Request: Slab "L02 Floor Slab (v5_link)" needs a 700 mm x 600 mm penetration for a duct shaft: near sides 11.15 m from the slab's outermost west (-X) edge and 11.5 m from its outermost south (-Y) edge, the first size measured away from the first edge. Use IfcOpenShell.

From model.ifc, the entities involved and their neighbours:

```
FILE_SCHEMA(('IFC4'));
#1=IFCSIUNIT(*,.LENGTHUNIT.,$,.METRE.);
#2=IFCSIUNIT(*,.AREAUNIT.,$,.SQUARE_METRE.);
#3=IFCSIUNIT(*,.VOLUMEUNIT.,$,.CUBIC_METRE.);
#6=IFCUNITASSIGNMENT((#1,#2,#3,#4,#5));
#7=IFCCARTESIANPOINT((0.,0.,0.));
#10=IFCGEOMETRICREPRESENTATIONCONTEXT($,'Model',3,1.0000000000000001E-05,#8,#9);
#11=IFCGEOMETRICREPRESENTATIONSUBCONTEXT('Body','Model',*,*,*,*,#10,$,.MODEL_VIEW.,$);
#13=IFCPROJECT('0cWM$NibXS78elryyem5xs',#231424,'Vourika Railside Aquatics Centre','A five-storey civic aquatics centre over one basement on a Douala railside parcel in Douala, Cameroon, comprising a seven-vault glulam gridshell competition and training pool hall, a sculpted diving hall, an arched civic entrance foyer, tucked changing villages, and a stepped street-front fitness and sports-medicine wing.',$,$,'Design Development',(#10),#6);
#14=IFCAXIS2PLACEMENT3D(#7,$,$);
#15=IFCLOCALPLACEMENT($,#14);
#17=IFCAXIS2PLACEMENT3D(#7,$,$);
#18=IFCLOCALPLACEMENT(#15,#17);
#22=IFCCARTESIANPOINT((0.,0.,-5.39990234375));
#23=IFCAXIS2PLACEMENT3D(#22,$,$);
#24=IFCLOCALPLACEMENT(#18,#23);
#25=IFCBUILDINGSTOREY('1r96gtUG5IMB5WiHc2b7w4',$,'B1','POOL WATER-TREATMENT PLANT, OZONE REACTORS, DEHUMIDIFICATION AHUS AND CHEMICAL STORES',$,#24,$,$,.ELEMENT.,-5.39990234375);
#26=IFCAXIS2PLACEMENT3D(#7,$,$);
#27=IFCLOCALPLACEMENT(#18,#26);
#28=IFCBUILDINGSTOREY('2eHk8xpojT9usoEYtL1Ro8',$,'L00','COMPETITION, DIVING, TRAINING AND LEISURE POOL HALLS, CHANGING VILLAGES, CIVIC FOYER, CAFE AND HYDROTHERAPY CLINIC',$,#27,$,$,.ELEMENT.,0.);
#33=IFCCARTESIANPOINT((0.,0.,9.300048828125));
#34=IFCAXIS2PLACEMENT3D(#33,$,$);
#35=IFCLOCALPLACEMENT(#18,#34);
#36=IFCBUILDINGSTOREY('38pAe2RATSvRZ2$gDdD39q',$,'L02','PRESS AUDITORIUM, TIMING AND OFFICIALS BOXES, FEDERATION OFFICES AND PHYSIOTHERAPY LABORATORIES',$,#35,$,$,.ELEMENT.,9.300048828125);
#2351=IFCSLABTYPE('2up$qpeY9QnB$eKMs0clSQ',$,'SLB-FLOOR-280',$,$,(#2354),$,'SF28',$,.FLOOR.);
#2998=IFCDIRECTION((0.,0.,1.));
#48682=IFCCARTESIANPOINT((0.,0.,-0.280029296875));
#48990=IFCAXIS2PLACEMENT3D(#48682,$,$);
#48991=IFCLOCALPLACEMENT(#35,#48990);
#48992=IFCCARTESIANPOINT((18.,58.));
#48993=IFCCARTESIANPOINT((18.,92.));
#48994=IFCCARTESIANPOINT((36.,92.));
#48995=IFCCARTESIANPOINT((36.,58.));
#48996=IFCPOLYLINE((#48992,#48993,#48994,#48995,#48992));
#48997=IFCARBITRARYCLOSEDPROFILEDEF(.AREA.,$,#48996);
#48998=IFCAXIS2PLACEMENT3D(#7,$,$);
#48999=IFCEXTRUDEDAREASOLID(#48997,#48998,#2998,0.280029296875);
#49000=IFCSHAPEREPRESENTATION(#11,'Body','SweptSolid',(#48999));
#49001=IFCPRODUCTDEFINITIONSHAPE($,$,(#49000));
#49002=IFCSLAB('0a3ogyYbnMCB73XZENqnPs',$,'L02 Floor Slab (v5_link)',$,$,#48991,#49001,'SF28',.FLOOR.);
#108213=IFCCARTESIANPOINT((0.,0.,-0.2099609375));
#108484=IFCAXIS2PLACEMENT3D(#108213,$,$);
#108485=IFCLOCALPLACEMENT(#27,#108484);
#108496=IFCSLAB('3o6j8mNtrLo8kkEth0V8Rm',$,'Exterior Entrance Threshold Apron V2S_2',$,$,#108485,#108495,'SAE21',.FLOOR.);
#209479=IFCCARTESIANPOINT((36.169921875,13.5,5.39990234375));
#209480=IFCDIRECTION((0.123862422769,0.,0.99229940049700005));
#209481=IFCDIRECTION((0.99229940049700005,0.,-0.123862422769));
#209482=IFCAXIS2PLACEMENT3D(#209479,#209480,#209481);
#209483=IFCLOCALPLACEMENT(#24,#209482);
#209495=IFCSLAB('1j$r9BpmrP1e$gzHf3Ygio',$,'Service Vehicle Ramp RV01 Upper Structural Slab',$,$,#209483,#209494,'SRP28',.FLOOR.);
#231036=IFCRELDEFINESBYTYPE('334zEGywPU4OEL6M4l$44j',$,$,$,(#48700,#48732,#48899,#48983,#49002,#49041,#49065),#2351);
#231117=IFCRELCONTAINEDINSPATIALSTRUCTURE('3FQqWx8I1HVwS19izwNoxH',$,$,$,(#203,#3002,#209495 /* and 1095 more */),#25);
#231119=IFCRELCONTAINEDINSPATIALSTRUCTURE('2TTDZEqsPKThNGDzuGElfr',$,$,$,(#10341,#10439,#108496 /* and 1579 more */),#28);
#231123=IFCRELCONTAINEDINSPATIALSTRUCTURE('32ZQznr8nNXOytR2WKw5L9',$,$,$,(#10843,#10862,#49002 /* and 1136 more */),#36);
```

```python
import numpy as np
import ifcopenshell
import ifcopenshell.api.feature
import ifcopenshell.api.geometry
import ifcopenshell.api.root
import ifcopenshell.geom
import ifcopenshell.util.placement
import ifcopenshell.util.representation
import ifcopenshell.util.shape
import ifcopenshell.util.unit

model = ifcopenshell.open("model.ifc")
unit_scale = ifcopenshell.util.unit.calculate_unit_scale(model)
settings = ifcopenshell.geom.settings()


def volume(element):
    """Net volume in cubic metres, openings subtracted."""
    shape = ifcopenshell.geom.create_shape(settings, element)
    return ifcopenshell.util.shape.get_volume(shape.geometry)


slab = model.by_guid("0a3ogyYbnMCB73XZENqnPs")
before = volume(slab)

# Extent in the slab's own axes, in metres. The edges named are its -X and -Y sides.
slab_shape = ifcopenshell.geom.create_shape(settings, slab)
vertices = ifcopenshell.util.shape.get_vertices(slab_shape.geometry)
x_min, y_min, bottom = vertices.min(axis=0)
top = vertices[:, 2].max()

opening = ifcopenshell.api.root.create_entity(model, ifc_class="IfcOpeningElement", name="Duct shaft opening", predefined_type="OPENING")
context = ifcopenshell.util.representation.get_context(model, "Model", "Body", "MODEL_VIEW")
width, depth = 0.7, 0.6
outline = [(0.0, 0.0), (width, 0.0), (width, depth), (0.0, depth), (0.0, 0.0)]
# Overshoot both faces by 50 mm so the cut is clean.
shape = ifcopenshell.api.geometry.add_slab_representation(
    model, context=context, depth=top - bottom + 0.1, polyline=outline
)
ifcopenshell.api.geometry.assign_representation(model, product=opening, representation=shape)

matrix = ifcopenshell.util.placement.get_local_placement(slab.ObjectPlacement)
matrix[:, 3] = matrix @ np.append(np.array([x_min + 11.15, y_min + 11.5, bottom - 0.05]) / unit_scale, 1.0)
ifcopenshell.api.geometry.edit_object_placement(model, product=opening, matrix=matrix, is_si=False)
ifcopenshell.api.feature.add_feature(model, feature=opening, element=slab)

after = volume(slab)

print(f"slab volume {before:.3f} -> {after:.3f} m3")

model.write("model_edited.ifc")
```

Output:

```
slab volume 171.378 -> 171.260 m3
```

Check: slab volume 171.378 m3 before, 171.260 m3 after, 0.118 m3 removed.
